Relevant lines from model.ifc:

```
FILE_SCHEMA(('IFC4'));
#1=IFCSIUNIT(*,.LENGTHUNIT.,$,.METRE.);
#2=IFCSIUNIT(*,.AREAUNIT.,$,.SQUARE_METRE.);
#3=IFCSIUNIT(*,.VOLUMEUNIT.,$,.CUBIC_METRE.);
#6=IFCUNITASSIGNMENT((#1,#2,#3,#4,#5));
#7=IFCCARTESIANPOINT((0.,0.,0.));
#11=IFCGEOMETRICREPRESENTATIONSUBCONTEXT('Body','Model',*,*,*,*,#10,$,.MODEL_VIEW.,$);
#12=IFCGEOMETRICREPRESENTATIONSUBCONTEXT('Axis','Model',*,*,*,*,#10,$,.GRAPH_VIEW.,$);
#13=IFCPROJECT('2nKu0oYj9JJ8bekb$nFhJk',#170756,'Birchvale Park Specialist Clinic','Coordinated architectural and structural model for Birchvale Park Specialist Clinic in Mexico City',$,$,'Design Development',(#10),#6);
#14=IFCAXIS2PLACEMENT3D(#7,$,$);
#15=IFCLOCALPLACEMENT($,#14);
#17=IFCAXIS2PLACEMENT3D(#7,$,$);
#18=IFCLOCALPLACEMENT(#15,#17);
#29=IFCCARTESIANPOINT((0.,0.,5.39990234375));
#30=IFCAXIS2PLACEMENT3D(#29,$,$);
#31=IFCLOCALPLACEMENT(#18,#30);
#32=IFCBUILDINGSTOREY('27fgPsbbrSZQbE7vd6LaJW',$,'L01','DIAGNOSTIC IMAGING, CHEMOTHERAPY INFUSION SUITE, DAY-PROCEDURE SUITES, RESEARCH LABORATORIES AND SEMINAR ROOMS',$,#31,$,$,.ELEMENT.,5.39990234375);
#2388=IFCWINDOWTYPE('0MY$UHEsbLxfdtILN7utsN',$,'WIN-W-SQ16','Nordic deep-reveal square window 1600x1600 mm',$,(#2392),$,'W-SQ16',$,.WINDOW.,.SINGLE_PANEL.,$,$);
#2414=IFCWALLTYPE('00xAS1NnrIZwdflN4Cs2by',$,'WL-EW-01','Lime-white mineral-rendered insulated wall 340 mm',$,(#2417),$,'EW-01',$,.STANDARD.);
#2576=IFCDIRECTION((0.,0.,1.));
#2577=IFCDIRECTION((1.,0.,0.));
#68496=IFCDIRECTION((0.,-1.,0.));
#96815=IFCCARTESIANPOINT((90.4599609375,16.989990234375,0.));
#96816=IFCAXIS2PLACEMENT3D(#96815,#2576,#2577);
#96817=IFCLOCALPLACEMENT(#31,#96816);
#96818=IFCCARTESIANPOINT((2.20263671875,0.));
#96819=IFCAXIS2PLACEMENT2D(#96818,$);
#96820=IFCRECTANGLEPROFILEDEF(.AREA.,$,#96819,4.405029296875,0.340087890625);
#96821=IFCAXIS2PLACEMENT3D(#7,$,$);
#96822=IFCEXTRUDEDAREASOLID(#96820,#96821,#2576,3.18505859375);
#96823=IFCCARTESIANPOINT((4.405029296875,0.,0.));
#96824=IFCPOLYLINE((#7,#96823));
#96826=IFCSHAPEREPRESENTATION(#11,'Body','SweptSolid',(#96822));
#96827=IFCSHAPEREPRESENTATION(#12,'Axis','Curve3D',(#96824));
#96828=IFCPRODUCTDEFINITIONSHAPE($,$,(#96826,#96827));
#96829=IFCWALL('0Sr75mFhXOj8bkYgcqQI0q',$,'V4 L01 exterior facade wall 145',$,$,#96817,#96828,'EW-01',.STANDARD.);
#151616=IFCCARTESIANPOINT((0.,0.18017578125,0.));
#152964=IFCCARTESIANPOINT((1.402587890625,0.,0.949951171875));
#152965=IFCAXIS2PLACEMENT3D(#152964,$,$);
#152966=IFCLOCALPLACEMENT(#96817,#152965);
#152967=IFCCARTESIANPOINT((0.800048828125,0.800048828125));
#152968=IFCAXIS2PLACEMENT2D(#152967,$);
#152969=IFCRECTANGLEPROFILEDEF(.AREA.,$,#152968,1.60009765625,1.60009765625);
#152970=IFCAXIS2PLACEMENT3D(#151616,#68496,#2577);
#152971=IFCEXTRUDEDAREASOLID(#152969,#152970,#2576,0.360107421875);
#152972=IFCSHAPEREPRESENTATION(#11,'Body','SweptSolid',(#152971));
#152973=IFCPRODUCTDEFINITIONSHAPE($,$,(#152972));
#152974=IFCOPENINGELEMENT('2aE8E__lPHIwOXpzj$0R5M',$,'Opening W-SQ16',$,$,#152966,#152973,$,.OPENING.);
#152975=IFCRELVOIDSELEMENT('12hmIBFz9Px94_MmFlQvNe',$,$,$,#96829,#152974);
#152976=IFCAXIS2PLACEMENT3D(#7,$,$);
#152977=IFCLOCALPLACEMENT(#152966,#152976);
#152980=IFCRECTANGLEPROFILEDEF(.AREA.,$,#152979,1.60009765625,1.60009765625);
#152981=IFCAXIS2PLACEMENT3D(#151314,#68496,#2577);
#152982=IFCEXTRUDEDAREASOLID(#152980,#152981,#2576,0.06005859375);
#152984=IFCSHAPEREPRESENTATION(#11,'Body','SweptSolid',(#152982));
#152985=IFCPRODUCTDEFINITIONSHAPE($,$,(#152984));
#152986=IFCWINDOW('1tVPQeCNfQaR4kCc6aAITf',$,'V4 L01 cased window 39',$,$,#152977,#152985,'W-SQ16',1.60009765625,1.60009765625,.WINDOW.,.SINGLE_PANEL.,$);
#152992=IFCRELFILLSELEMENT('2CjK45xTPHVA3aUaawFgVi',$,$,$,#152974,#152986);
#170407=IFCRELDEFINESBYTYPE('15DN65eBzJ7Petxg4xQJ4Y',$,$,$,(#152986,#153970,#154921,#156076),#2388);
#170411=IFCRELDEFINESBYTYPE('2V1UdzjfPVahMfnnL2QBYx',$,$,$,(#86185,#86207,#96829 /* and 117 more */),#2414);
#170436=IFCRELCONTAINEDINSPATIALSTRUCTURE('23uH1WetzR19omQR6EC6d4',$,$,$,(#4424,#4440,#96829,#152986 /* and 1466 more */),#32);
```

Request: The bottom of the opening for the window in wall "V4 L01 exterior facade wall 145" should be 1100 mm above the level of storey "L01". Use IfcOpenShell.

```python
import numpy as np
import ifcopenshell
import ifcopenshell.api.geometry
import ifcopenshell.geom
import ifcopenshell.util.element
import ifcopenshell.util.placement
import ifcopenshell.util.shape
import ifcopenshell.util.unit

model = ifcopenshell.open("model.ifc")
unit_scale = ifcopenshell.util.unit.calculate_unit_scale(model)

window = model.by_guid("1tVPQeCNfQaR4kCc6aAITf")
opening = window.FillsVoids[0].RelatingOpeningElement
storey = ifcopenshell.util.element.get_container(window, ifc_class="IfcBuildingStorey")
level = ifcopenshell.util.placement.get_local_placement(storey.ObjectPlacement)[2, 3]

# The opening's origin need not be at the sill, so measure its lowest point.
shape = ifcopenshell.geom.create_shape(ifcopenshell.geom.settings(), opening)
bottom = ifcopenshell.util.shape.get_shape_bottom_elevation(shape, shape.geometry) / unit_scale
dz = level + 1.1 - bottom

shift = np.array([0.0, 0.0, dz])
# The window is placed relative to its opening, so it follows when the opening moves.
matrix = ifcopenshell.util.placement.get_local_placement(opening.ObjectPlacement)
matrix[:3, 3] += shift
ifcopenshell.api.geometry.edit_object_placement(
    model, product=opening, matrix=matrix, is_si=False, should_transform_children=True
)

print(f"moved by {dz * unit_scale:+.3f} m")

model.write("model_rev.ifc")
```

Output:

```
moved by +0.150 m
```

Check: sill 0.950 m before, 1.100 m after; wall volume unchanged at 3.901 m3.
